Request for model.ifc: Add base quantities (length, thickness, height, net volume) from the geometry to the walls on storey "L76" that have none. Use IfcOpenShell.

First a look at what the model holds.

```python
import ifcopenshell
import ifcopenshell.util.element
import ifcopenshell.util.unit

model = ifcopenshell.open("model.ifc")
print(model.schema)
for unit_type in ("LENGTHUNIT", "AREAUNIT", "VOLUMEUNIT"):
    print(unit_type, ifcopenshell.util.unit.calculate_unit_scale(model, unit_type))
storey = next(s for s in model.by_type("IfcBuildingStorey") if s.Name == "L76")
walls = [e for e in ifcopenshell.util.element.get_decomposition(storey) if e.is_a("IfcWall")]
for e in sorted(walls, key=lambda e: e.id()):
    print(e.id(), e.is_a(), e.Name, list(ifcopenshell.util.element.get_psets(e, qtos_only=True)), sep=" | ")
```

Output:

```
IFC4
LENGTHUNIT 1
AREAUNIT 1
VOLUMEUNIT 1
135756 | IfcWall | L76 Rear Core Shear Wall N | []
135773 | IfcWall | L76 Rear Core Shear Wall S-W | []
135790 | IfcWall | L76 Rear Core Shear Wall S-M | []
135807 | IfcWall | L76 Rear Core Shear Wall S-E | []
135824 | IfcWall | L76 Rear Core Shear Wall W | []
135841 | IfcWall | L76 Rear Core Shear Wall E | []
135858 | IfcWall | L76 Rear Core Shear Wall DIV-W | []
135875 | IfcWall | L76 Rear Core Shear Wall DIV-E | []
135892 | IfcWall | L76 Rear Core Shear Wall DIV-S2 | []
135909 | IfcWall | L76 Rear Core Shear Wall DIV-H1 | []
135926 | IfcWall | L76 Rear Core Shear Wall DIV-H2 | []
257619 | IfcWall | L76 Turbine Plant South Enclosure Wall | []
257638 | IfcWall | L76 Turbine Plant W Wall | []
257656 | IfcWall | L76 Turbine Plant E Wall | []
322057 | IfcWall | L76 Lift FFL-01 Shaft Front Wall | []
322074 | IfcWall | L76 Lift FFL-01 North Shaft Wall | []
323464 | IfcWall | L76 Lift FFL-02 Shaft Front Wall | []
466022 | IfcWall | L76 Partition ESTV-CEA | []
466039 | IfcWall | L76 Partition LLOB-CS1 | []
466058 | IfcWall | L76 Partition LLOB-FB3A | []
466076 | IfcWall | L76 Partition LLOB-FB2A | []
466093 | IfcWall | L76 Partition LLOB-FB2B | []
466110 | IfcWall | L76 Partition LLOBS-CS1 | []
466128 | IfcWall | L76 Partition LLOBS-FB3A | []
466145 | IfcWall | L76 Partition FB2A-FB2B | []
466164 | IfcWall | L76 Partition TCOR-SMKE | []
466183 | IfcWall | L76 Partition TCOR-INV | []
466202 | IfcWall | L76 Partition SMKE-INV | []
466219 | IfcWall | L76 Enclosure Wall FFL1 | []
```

```python
import ifcopenshell
import ifcopenshell.api.pset
import ifcopenshell.geom
import ifcopenshell.util.element
import ifcopenshell.util.shape
import ifcopenshell.util.unit

model = ifcopenshell.open("model.ifc")
unit_scale = ifcopenshell.util.unit.calculate_unit_scale(model)
volume_scale = ifcopenshell.util.unit.calculate_unit_scale(model, "VOLUMEUNIT")
settings = ifcopenshell.geom.settings()

storey = next(s for s in model.by_type("IfcBuildingStorey") if s.Name == "L76")
walls = [e for e in ifcopenshell.util.element.get_decomposition(storey) if e.is_a("IfcWall")]

for e in sorted(walls, key=lambda e: e.id()):
    if ifcopenshell.util.element.get_psets(e, qtos_only=True, should_inherit=False):
        continue
    # Geometry comes back in metres, in the element's own axes.
    shape = ifcopenshell.geom.create_shape(settings, e)
    values = {
        "Length": ifcopenshell.util.shape.get_x(shape.geometry) / unit_scale,
        "Width": ifcopenshell.util.shape.get_y(shape.geometry) / unit_scale,
        "Height": ifcopenshell.util.shape.get_z(shape.geometry) / unit_scale,
        "NetVolume": ifcopenshell.util.shape.get_volume(shape.geometry) / volume_scale,
    }
    qto = ifcopenshell.api.pset.add_qto(model, product=e, name="Qto_WallBaseQuantities")
    ifcopenshell.api.pset.edit_qto(model, qto=qto, properties=values)
    print(e.id(), {k: round(v, 3) for k, v in values.items()})

model.write("model_rev.ifc")
```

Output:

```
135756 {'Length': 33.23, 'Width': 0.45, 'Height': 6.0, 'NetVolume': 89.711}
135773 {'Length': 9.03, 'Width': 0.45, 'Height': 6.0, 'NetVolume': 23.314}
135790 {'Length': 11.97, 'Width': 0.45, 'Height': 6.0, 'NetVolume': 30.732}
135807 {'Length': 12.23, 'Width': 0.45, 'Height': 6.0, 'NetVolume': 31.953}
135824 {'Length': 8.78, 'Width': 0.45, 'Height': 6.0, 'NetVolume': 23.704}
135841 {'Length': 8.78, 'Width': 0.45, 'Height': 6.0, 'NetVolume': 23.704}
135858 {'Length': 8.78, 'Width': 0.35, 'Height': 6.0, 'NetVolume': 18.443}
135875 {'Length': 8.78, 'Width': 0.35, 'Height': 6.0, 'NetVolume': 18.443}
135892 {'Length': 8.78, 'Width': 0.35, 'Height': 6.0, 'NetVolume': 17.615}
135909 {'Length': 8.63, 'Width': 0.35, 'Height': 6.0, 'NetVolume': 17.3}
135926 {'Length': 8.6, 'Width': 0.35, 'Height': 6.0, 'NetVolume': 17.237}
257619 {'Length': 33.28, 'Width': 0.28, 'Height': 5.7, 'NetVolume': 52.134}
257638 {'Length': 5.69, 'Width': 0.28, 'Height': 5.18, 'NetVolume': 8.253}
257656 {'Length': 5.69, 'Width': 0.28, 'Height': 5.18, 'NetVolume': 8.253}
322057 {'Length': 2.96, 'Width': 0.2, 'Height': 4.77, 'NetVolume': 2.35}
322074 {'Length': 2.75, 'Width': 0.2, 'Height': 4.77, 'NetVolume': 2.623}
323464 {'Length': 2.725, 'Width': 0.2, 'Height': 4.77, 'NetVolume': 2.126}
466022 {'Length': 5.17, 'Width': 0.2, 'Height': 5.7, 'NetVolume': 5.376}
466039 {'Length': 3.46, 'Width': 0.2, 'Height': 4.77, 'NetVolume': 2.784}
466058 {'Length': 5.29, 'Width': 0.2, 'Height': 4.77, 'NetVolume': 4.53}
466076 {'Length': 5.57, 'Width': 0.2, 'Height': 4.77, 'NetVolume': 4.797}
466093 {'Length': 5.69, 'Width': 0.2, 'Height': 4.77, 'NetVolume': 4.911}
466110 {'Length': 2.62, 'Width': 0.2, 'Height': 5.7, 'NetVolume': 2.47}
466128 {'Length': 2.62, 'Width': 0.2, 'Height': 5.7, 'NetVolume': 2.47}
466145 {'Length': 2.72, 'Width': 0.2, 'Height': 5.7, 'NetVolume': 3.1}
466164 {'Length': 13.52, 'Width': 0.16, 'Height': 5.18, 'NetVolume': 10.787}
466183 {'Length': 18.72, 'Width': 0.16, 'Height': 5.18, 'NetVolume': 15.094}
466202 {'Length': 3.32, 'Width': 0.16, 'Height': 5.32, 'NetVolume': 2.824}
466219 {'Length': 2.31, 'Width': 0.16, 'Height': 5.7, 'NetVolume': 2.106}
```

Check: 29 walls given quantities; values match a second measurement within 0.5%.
